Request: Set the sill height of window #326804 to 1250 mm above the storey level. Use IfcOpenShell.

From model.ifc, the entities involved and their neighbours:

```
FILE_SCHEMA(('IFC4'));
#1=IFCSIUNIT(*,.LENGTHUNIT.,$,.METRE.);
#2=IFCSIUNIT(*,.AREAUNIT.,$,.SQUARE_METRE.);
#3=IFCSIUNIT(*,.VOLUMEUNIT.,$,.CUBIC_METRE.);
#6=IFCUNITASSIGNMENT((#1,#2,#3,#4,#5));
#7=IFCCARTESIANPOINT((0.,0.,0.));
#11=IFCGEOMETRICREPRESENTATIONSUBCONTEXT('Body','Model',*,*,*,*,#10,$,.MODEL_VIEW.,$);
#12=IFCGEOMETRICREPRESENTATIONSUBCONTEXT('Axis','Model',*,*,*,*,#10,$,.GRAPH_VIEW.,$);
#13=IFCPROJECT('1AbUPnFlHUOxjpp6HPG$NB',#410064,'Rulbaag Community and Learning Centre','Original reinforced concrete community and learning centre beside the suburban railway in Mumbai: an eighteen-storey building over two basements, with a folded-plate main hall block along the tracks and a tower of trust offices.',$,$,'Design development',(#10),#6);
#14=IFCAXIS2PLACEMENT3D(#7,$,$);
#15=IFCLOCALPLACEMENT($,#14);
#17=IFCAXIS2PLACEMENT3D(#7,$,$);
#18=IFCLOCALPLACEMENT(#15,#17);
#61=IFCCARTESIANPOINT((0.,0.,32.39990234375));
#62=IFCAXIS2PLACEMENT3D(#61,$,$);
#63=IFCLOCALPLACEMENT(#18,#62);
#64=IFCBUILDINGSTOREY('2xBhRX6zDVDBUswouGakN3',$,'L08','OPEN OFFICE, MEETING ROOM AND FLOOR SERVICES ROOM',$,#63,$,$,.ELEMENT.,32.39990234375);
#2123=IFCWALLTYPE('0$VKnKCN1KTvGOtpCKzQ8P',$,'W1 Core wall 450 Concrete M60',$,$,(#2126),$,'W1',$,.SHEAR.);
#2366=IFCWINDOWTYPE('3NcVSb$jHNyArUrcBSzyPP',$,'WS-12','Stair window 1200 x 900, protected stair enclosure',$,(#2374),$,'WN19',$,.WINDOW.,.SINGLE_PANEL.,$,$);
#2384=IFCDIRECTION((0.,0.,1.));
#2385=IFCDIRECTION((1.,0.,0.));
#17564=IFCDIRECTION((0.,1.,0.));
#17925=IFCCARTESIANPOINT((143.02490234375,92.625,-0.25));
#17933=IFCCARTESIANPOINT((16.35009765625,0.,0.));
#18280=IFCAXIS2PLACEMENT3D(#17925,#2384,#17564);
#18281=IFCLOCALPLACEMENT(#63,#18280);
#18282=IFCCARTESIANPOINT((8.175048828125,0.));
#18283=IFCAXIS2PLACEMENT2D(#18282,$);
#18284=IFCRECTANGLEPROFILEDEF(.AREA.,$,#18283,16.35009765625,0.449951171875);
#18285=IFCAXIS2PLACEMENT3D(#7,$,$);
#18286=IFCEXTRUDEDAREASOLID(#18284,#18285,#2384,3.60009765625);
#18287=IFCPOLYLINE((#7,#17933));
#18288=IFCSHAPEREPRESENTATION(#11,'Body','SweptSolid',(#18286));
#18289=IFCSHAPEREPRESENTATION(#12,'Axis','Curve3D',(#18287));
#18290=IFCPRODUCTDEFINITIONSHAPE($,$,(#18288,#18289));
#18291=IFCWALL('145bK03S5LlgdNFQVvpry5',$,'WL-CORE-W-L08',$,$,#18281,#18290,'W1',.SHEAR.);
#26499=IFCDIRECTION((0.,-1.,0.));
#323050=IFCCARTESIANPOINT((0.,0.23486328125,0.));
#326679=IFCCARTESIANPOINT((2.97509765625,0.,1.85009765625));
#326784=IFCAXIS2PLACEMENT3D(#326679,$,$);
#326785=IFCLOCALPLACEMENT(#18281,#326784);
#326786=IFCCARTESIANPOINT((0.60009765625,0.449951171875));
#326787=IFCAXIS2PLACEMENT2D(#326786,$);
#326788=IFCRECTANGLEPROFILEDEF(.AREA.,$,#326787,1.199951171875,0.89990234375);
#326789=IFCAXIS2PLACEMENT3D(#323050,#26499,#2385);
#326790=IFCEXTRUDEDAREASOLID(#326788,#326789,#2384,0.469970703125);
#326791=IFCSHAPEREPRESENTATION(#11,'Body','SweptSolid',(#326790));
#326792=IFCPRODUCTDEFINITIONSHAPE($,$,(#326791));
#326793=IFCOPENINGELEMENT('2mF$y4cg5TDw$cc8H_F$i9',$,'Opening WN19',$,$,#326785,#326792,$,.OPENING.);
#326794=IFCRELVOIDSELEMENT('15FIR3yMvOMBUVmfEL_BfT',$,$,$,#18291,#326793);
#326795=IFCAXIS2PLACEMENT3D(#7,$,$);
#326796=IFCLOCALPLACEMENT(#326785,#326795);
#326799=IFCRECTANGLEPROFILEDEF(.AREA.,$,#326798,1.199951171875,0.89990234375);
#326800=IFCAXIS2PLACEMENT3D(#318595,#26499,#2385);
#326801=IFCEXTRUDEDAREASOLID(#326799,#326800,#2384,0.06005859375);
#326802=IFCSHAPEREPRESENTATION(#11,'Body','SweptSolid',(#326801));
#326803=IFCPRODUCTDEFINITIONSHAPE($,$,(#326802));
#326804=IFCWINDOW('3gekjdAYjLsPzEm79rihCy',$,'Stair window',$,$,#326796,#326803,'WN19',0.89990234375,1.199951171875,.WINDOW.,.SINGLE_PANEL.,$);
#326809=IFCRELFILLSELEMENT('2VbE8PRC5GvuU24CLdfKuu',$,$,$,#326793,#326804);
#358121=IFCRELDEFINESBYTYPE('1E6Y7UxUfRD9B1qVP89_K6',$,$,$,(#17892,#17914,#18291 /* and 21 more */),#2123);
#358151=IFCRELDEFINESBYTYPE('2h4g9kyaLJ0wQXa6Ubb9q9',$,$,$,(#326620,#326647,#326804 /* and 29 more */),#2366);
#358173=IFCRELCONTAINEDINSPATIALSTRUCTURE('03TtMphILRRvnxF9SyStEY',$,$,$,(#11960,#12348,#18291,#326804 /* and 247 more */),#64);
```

```python
import numpy as np
import ifcopenshell
import ifcopenshell.api.geometry
import ifcopenshell.geom
import ifcopenshell.util.element
import ifcopenshell.util.placement
import ifcopenshell.util.shape
import ifcopenshell.util.unit

model = ifcopenshell.open("model.ifc")
unit_scale = ifcopenshell.util.unit.calculate_unit_scale(model)

window = model.by_guid("3gekjdAYjLsPzEm79rihCy")
opening = window.FillsVoids[0].RelatingOpeningElement
storey = ifcopenshell.util.element.get_container(window, ifc_class="IfcBuildingStorey")
level = ifcopenshell.util.placement.get_local_placement(storey.ObjectPlacement)[2, 3]

# The opening's origin need not be at the sill, so measure its lowest point.
shape = ifcopenshell.geom.create_shape(ifcopenshell.geom.settings(), opening)
bottom = ifcopenshell.util.shape.get_shape_bottom_elevation(shape, shape.geometry) / unit_scale
dz = level + 1.25 / unit_scale - bottom

shift = np.array([0.0, 0.0, dz])
# The window is placed relative to its opening, so it follows when the opening moves.
matrix = ifcopenshell.util.placement.get_local_placement(opening.ObjectPlacement)
matrix[:3, 3] += shift
ifcopenshell.api.geometry.edit_object_placement(
    model, product=opening, matrix=matrix, is_si=False, should_transform_children=True
)

print(f"moved by {dz * unit_scale:+.3f} m")

model.write("model_v2.ifc")
```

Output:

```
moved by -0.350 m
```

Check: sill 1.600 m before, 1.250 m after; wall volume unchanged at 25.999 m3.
